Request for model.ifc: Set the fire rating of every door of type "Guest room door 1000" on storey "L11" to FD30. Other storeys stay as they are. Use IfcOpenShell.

First a look at what the model holds.

```python
import ifcopenshell
import ifcopenshell.util.element

model = ifcopenshell.open("model.ifc")
print(model.schema)
storey = next(s for s in model.by_type("IfcBuildingStorey") if s.Name == "L11")
doors = [e for e in ifcopenshell.util.element.get_decomposition(storey) if e.is_a("IfcDoor")]
seen = {}
for e in doors:
    element_type = ifcopenshell.util.element.get_type(e)
    key = (element_type.Name if element_type != e and element_type else None, ifcopenshell.util.element.get_pset(e, "Pset_DoorCommon", "FireRating"))
    seen[key] = seen.get(key, 0) + 1
for (name, value), count in sorted(seen.items(), key=str):
    print(count, "x", name, "|", value)
```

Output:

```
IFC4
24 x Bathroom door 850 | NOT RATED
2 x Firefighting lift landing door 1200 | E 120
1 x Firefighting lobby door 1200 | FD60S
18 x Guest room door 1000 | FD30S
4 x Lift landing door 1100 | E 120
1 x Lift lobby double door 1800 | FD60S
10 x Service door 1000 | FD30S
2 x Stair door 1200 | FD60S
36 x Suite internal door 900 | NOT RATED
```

```python
import ifcopenshell
import ifcopenshell.api.pset
import ifcopenshell.util.element

model = ifcopenshell.open("model.ifc")

storey = next(s for s in model.by_type("IfcBuildingStorey") if s.Name == "L11")
doors = [e for e in ifcopenshell.util.element.get_decomposition(storey) if e.is_a("IfcDoor")]

count = 0
for e in doors:
    element_type = ifcopenshell.util.element.get_type(e)
    if element_type in (None, e) or element_type.Name != "Guest room door 1000":
        continue
    found = ifcopenshell.util.element.get_pset(e, "Pset_DoorCommon", should_inherit=False)
    if found:
        pset = model.by_id(found["id"])
        if len(ifcopenshell.util.element.get_elements_by_pset(pset)) > 1:
            pset = ifcopenshell.api.pset.unshare_pset(model, products=[e], pset=pset)[0]
    else:
        pset = ifcopenshell.api.pset.add_pset(model, product=e, name="Pset_DoorCommon")
    ifcopenshell.api.pset.edit_pset(model, pset=pset, properties={"FireRating": "FD30"})
    count += 1

print(count, "doors updated")

model.write("model_v2.ifc")
```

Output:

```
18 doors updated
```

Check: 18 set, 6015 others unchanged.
